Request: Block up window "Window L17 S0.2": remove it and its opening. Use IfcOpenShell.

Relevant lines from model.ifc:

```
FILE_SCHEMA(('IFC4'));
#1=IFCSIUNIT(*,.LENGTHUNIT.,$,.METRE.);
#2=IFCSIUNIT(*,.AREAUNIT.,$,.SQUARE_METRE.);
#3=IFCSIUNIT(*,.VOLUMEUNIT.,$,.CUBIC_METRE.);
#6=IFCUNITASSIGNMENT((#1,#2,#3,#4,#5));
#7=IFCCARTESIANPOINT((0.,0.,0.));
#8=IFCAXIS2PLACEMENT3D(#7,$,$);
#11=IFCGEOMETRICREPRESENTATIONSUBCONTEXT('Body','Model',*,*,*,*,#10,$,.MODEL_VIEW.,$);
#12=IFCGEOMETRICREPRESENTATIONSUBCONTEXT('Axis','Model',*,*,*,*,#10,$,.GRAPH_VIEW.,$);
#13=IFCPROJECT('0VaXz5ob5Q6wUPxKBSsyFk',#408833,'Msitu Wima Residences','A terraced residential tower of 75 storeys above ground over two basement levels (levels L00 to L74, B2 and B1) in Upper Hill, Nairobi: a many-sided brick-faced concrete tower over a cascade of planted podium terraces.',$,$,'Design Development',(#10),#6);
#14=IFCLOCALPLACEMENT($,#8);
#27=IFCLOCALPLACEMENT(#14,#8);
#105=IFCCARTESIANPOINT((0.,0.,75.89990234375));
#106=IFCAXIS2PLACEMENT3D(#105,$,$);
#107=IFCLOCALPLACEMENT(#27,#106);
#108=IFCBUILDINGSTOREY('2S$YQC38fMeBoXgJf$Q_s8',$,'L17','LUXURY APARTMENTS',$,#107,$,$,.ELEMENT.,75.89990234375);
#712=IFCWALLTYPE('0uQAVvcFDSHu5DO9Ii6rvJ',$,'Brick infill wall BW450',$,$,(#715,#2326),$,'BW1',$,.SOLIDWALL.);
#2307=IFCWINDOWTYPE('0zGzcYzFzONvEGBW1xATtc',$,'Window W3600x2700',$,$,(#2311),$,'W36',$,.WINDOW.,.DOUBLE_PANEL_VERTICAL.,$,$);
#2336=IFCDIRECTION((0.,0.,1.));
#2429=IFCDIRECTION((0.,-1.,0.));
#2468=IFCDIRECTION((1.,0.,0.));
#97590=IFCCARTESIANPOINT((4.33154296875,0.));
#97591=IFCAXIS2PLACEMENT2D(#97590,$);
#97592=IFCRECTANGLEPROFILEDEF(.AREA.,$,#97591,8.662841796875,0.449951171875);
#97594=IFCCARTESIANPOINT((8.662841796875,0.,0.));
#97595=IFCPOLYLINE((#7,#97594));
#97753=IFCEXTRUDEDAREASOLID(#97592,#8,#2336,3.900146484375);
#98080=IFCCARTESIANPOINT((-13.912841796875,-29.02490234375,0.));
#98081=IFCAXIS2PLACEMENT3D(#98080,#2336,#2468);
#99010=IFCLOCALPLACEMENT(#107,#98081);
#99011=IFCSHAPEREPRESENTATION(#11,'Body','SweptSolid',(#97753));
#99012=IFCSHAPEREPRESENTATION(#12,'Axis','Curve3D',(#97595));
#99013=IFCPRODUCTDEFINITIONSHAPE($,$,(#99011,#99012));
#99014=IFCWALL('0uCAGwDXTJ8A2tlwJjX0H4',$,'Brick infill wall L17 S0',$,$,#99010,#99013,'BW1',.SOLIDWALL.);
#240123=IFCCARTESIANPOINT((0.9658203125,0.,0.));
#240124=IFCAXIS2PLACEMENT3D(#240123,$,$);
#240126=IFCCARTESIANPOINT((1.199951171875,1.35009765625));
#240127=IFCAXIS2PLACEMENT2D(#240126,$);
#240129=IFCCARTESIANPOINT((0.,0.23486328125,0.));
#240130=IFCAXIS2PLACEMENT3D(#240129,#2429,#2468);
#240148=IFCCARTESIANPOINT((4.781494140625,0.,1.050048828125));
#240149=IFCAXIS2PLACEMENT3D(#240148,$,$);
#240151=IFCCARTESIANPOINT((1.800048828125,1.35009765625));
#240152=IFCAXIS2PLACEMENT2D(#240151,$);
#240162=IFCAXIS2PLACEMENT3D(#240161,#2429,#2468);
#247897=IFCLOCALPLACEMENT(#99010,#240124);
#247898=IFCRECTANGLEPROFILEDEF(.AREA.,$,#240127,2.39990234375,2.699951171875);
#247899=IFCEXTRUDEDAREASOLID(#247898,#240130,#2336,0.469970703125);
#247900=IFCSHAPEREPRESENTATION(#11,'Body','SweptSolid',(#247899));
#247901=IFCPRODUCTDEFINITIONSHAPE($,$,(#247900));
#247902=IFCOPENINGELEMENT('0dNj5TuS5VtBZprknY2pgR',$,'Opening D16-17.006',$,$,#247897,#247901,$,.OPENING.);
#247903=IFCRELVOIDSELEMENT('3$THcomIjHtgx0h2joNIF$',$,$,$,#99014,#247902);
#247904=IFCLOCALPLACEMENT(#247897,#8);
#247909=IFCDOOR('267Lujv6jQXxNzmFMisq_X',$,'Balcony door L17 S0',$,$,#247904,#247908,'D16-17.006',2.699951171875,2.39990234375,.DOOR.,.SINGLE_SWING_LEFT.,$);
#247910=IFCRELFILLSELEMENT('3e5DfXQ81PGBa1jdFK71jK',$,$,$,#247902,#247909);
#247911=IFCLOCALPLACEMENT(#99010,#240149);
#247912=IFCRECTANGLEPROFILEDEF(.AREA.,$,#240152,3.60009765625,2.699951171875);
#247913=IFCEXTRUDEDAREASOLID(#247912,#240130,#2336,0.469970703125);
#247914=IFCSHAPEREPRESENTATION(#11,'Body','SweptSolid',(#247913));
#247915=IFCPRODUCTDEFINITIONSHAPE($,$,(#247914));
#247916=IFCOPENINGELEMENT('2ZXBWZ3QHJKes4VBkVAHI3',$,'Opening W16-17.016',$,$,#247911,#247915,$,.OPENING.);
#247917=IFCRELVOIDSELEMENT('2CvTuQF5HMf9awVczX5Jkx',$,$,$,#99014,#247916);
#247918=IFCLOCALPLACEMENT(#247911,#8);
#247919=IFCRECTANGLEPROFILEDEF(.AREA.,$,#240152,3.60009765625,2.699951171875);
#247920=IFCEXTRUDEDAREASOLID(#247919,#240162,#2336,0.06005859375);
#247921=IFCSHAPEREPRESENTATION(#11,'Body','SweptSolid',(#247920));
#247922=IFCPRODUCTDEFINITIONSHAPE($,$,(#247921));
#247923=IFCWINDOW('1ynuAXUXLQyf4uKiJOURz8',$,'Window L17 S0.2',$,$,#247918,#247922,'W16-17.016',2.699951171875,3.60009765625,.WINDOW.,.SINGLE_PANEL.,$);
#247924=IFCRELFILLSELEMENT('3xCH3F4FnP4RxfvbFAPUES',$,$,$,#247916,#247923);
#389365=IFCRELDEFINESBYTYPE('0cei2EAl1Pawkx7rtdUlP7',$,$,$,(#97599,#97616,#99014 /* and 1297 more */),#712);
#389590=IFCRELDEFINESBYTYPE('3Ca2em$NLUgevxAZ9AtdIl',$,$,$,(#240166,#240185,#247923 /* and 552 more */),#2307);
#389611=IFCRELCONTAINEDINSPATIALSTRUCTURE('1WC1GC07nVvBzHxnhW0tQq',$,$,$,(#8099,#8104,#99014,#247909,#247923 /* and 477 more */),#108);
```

```python
import ifcopenshell
import ifcopenshell.api.feature
import ifcopenshell.api.root
import ifcopenshell.geom
import ifcopenshell.util.shape

model = ifcopenshell.open("model.ifc")
settings = ifcopenshell.geom.settings()


def volume(element):
    """Net volume in cubic metres, openings subtracted."""
    shape = ifcopenshell.geom.create_shape(settings, element)
    return ifcopenshell.util.shape.get_volume(shape.geometry)


window = model.by_guid("1ynuAXUXLQyf4uKiJOURz8")
opening = window.FillsVoids[0].RelatingOpeningElement
wall = opening.VoidsElements[0].RelatingBuildingElement
before = volume(wall)

ifcopenshell.api.root.remove_product(model, product=window)
ifcopenshell.api.feature.remove_feature(model, feature=opening)

after = volume(wall)

print(f"wall volume {before:.3f} -> {after:.3f} m3")

model.write("model-out.ifc")
```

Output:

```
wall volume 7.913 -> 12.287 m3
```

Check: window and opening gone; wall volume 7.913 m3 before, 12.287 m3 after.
